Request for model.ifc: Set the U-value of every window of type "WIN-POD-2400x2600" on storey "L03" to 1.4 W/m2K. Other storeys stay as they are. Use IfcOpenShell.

First a look at what the model holds.

```python
import ifcopenshell
import ifcopenshell.util.element

model = ifcopenshell.open("model.ifc")
print(model.schema)
storey = next(s for s in model.by_type("IfcBuildingStorey") if s.Name == "L03")
windows = [e for e in ifcopenshell.util.element.get_decomposition(storey) if e.is_a("IfcWindow")]
seen = {}
for e in windows:
    element_type = ifcopenshell.util.element.get_type(e)
    key = (element_type.Name if element_type != e and element_type else None, ifcopenshell.util.element.get_pset(e, "Pset_WindowCommon", "ThermalTransmittance"))
    seen[key] = seen.get(key, 0) + 1
for (name, value), count in sorted(seen.items(), key=str):
    print(count, "x", name, "|", value)
```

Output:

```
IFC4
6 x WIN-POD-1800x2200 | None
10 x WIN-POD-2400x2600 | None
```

```python
import ifcopenshell
import ifcopenshell.api.pset
import ifcopenshell.util.element

model = ifcopenshell.open("model.ifc")

storey = next(s for s in model.by_type("IfcBuildingStorey") if s.Name == "L03")
windows = [e for e in ifcopenshell.util.element.get_decomposition(storey) if e.is_a("IfcWindow")]

count = 0
for e in windows:
    element_type = ifcopenshell.util.element.get_type(e)
    if element_type in (None, e) or element_type.Name != "WIN-POD-2400x2600":
        continue
    # add_pset returns the element's existing set when there is one.
    pset = ifcopenshell.api.pset.add_pset(model, product=e, name="Pset_WindowCommon")
    ifcopenshell.api.pset.edit_pset(model, pset=pset, properties={"ThermalTransmittance": 1.4})
    count += 1

print(count, "windows updated")

model.write("model_rev.ifc")
```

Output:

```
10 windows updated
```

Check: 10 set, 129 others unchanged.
